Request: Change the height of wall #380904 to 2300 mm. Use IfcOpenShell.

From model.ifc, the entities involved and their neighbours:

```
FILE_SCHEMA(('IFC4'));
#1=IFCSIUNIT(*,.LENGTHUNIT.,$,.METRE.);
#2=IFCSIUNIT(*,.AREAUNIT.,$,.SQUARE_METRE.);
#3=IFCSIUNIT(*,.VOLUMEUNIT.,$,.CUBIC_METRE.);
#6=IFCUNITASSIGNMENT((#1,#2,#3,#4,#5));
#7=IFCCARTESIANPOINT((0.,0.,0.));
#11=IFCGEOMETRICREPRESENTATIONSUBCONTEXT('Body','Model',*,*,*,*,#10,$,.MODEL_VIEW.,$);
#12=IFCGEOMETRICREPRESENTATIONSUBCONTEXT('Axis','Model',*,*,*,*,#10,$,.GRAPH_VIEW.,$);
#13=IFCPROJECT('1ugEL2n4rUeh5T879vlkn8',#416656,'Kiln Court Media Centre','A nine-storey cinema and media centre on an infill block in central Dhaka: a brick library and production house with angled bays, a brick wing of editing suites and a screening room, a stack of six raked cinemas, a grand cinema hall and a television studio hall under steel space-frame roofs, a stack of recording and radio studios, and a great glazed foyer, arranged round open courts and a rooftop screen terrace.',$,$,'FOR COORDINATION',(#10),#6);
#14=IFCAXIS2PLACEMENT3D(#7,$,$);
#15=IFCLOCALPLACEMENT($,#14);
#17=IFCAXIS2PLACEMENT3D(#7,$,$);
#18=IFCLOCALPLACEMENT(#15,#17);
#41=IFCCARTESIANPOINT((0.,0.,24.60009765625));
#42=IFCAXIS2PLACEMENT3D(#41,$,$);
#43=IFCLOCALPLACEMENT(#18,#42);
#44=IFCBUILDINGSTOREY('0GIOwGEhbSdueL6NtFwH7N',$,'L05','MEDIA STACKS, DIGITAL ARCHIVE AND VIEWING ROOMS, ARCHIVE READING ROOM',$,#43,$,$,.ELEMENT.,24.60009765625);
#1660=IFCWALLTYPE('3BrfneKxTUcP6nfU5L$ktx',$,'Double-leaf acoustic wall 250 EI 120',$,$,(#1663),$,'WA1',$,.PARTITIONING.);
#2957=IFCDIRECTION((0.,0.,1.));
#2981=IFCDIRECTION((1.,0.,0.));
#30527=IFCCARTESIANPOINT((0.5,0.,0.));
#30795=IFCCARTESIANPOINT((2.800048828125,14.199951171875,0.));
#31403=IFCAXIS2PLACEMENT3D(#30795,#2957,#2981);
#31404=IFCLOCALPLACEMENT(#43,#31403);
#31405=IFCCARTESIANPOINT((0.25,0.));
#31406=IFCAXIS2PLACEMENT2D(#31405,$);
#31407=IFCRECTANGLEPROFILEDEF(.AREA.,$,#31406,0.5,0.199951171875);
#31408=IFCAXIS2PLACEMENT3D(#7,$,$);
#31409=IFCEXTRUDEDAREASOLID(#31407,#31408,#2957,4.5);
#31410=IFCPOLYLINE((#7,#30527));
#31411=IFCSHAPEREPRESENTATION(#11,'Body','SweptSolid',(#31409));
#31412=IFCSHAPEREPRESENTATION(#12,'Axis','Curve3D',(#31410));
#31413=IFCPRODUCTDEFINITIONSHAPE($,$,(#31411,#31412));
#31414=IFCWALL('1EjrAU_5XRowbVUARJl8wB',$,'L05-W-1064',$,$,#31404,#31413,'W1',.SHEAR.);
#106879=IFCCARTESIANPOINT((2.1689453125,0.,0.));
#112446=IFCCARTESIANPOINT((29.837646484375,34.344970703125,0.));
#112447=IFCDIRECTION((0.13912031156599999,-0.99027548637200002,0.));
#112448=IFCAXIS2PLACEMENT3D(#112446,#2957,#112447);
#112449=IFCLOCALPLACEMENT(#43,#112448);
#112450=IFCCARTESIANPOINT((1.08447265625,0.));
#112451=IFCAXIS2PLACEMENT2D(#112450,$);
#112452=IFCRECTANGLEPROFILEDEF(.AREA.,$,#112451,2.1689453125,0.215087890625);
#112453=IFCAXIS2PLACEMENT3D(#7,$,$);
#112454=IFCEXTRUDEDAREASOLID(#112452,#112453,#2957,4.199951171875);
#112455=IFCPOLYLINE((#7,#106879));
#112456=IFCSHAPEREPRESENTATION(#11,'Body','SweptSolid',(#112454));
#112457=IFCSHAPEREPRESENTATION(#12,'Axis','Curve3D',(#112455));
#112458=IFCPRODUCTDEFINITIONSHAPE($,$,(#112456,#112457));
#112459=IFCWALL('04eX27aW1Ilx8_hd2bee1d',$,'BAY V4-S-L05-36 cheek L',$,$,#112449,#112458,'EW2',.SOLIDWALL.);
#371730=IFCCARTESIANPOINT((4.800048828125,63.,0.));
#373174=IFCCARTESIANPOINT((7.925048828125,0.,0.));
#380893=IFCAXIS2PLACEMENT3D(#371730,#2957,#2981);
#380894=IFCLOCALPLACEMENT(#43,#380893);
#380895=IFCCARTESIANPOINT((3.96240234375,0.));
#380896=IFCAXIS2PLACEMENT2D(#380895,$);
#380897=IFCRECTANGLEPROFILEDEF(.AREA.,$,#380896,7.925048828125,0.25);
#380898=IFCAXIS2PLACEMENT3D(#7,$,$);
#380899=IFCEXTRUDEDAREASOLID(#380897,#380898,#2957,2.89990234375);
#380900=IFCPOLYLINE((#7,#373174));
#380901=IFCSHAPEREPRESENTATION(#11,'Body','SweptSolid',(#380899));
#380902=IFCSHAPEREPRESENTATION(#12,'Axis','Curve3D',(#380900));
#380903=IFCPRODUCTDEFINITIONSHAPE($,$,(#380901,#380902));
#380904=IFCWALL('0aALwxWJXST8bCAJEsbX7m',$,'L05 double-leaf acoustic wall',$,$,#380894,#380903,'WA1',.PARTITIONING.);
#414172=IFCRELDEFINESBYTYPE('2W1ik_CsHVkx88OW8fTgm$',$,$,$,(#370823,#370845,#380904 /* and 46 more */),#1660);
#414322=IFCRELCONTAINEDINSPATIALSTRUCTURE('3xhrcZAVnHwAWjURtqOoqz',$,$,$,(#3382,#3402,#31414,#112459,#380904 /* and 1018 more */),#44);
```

```python
import ifcopenshell
import ifcopenshell.geom
import ifcopenshell.util.representation
import ifcopenshell.util.shape
import ifcopenshell.util.unit

model = ifcopenshell.open("model.ifc")
unit_scale = ifcopenshell.util.unit.calculate_unit_scale(model)
settings = ifcopenshell.geom.settings()


def volume(element):
    """Net volume in cubic metres, openings subtracted."""
    shape = ifcopenshell.geom.create_shape(settings, element)
    return ifcopenshell.util.shape.get_volume(shape.geometry)


wall = model.by_id(380904)
before = volume(wall)

body = ifcopenshell.util.representation.get_representation(wall, "Model", "Body")
solid = body.Items[0]
old_height = solid.Depth
solid.Depth = 2.3 / unit_scale
after = volume(wall)

print(f"height {old_height:g} -> {solid.Depth:g}, volume {before:.3f} -> {after:.3f} m3")

model.write("model-out.ifc")
```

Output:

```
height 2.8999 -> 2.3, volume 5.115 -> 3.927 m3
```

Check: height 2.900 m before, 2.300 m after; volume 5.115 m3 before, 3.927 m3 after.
